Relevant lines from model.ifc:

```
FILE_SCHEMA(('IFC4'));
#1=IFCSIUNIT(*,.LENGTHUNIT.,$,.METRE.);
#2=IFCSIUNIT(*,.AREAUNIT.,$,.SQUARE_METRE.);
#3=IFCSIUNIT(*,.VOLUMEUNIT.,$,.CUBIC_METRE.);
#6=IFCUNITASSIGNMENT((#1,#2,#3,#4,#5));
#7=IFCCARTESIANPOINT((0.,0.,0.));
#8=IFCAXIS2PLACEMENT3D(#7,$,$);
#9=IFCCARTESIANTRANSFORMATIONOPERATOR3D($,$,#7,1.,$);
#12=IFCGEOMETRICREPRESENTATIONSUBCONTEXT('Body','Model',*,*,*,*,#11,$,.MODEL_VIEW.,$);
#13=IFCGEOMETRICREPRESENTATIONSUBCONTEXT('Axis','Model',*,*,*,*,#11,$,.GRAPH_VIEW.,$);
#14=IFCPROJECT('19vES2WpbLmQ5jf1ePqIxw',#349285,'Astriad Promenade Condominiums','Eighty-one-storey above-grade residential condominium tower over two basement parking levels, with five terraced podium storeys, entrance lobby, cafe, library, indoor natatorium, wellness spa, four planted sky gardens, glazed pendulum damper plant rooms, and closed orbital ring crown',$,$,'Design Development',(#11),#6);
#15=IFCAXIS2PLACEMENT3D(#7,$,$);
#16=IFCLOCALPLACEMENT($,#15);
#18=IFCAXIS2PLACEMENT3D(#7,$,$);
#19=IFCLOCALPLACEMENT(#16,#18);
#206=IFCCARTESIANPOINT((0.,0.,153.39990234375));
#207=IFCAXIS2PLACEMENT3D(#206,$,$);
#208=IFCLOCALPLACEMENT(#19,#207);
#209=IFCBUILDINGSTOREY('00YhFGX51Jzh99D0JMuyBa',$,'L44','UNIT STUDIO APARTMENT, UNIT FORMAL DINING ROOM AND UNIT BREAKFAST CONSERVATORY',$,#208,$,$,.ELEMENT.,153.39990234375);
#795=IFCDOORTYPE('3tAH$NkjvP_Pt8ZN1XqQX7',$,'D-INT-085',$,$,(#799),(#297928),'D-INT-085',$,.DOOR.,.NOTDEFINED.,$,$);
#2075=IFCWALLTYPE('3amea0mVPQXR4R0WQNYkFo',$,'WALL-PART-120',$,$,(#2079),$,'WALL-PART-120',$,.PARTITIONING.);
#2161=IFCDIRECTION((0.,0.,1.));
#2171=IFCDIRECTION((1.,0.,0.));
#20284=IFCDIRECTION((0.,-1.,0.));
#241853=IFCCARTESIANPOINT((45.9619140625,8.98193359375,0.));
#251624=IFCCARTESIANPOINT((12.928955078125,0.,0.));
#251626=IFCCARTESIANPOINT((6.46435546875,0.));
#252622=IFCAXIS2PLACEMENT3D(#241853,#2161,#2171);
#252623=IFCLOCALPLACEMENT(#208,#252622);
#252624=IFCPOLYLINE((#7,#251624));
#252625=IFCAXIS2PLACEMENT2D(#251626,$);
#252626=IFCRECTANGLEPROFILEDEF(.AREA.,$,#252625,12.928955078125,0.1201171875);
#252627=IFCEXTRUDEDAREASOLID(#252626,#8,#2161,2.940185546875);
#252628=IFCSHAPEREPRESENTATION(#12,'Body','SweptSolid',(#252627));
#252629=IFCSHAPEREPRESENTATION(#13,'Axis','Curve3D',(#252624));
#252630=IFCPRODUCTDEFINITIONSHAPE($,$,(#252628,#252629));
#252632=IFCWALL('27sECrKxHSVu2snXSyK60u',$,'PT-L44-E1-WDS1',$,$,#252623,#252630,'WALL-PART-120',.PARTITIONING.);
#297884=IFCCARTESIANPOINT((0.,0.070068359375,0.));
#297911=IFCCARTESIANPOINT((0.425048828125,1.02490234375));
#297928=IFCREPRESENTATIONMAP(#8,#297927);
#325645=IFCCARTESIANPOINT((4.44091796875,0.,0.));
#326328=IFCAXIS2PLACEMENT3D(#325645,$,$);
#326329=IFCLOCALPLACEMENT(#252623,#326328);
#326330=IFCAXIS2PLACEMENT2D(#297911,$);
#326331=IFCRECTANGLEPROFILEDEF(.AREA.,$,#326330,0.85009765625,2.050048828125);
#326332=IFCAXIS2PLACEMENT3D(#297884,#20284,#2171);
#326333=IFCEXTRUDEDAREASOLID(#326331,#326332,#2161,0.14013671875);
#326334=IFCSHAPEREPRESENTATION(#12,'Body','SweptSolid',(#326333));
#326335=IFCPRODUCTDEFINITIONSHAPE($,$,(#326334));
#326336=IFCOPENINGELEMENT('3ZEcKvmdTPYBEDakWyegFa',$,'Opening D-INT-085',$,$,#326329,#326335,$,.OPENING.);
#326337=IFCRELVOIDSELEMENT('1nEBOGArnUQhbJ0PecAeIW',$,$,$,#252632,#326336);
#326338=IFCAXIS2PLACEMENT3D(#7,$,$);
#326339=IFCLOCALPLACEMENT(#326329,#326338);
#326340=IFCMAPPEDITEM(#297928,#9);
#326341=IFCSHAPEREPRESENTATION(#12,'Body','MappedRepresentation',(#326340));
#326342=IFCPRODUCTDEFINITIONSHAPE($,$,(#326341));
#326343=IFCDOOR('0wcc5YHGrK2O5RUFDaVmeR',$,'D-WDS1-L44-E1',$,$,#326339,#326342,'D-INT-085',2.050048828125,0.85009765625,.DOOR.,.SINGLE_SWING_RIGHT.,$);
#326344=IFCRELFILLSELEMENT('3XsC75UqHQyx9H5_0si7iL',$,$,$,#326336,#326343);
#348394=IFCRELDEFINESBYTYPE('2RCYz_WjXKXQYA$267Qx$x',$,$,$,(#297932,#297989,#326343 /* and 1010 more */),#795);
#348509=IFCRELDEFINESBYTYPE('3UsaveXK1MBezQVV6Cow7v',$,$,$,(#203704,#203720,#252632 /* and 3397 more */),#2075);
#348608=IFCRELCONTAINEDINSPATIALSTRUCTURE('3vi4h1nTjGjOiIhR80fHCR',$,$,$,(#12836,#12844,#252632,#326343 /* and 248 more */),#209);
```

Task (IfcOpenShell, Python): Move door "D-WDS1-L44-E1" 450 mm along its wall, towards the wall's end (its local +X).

```python
import ifcopenshell
import ifcopenshell.api.geometry
import ifcopenshell.util.placement
import ifcopenshell.util.unit

model = ifcopenshell.open("model.ifc")
unit_scale = ifcopenshell.util.unit.calculate_unit_scale(model)

door = model.by_guid("0wcc5YHGrK2O5RUFDaVmeR")
opening = door.FillsVoids[0].RelatingOpeningElement
wall = opening.VoidsElements[0].RelatingBuildingElement

wall_matrix = ifcopenshell.util.placement.get_local_placement(wall.ObjectPlacement)
shift = wall_matrix[:3, 0] * 0.45 / unit_scale
before = ifcopenshell.util.placement.get_local_placement(door.ObjectPlacement)[:3, 3].copy()

# The door is placed relative to its opening, so it follows when the opening moves.
matrix = ifcopenshell.util.placement.get_local_placement(opening.ObjectPlacement)
matrix[:3, 3] += shift
ifcopenshell.api.geometry.edit_object_placement(
    model, product=opening, matrix=matrix, is_si=False, should_transform_children=True
)

after = ifcopenshell.util.placement.get_local_placement(door.ObjectPlacement)[:3, 3]
print("door moved by", (after - before).round(3) + 0.0)

model.write("model_updated.ifc")
```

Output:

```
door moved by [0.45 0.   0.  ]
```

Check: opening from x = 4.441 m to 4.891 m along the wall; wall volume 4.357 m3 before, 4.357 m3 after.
